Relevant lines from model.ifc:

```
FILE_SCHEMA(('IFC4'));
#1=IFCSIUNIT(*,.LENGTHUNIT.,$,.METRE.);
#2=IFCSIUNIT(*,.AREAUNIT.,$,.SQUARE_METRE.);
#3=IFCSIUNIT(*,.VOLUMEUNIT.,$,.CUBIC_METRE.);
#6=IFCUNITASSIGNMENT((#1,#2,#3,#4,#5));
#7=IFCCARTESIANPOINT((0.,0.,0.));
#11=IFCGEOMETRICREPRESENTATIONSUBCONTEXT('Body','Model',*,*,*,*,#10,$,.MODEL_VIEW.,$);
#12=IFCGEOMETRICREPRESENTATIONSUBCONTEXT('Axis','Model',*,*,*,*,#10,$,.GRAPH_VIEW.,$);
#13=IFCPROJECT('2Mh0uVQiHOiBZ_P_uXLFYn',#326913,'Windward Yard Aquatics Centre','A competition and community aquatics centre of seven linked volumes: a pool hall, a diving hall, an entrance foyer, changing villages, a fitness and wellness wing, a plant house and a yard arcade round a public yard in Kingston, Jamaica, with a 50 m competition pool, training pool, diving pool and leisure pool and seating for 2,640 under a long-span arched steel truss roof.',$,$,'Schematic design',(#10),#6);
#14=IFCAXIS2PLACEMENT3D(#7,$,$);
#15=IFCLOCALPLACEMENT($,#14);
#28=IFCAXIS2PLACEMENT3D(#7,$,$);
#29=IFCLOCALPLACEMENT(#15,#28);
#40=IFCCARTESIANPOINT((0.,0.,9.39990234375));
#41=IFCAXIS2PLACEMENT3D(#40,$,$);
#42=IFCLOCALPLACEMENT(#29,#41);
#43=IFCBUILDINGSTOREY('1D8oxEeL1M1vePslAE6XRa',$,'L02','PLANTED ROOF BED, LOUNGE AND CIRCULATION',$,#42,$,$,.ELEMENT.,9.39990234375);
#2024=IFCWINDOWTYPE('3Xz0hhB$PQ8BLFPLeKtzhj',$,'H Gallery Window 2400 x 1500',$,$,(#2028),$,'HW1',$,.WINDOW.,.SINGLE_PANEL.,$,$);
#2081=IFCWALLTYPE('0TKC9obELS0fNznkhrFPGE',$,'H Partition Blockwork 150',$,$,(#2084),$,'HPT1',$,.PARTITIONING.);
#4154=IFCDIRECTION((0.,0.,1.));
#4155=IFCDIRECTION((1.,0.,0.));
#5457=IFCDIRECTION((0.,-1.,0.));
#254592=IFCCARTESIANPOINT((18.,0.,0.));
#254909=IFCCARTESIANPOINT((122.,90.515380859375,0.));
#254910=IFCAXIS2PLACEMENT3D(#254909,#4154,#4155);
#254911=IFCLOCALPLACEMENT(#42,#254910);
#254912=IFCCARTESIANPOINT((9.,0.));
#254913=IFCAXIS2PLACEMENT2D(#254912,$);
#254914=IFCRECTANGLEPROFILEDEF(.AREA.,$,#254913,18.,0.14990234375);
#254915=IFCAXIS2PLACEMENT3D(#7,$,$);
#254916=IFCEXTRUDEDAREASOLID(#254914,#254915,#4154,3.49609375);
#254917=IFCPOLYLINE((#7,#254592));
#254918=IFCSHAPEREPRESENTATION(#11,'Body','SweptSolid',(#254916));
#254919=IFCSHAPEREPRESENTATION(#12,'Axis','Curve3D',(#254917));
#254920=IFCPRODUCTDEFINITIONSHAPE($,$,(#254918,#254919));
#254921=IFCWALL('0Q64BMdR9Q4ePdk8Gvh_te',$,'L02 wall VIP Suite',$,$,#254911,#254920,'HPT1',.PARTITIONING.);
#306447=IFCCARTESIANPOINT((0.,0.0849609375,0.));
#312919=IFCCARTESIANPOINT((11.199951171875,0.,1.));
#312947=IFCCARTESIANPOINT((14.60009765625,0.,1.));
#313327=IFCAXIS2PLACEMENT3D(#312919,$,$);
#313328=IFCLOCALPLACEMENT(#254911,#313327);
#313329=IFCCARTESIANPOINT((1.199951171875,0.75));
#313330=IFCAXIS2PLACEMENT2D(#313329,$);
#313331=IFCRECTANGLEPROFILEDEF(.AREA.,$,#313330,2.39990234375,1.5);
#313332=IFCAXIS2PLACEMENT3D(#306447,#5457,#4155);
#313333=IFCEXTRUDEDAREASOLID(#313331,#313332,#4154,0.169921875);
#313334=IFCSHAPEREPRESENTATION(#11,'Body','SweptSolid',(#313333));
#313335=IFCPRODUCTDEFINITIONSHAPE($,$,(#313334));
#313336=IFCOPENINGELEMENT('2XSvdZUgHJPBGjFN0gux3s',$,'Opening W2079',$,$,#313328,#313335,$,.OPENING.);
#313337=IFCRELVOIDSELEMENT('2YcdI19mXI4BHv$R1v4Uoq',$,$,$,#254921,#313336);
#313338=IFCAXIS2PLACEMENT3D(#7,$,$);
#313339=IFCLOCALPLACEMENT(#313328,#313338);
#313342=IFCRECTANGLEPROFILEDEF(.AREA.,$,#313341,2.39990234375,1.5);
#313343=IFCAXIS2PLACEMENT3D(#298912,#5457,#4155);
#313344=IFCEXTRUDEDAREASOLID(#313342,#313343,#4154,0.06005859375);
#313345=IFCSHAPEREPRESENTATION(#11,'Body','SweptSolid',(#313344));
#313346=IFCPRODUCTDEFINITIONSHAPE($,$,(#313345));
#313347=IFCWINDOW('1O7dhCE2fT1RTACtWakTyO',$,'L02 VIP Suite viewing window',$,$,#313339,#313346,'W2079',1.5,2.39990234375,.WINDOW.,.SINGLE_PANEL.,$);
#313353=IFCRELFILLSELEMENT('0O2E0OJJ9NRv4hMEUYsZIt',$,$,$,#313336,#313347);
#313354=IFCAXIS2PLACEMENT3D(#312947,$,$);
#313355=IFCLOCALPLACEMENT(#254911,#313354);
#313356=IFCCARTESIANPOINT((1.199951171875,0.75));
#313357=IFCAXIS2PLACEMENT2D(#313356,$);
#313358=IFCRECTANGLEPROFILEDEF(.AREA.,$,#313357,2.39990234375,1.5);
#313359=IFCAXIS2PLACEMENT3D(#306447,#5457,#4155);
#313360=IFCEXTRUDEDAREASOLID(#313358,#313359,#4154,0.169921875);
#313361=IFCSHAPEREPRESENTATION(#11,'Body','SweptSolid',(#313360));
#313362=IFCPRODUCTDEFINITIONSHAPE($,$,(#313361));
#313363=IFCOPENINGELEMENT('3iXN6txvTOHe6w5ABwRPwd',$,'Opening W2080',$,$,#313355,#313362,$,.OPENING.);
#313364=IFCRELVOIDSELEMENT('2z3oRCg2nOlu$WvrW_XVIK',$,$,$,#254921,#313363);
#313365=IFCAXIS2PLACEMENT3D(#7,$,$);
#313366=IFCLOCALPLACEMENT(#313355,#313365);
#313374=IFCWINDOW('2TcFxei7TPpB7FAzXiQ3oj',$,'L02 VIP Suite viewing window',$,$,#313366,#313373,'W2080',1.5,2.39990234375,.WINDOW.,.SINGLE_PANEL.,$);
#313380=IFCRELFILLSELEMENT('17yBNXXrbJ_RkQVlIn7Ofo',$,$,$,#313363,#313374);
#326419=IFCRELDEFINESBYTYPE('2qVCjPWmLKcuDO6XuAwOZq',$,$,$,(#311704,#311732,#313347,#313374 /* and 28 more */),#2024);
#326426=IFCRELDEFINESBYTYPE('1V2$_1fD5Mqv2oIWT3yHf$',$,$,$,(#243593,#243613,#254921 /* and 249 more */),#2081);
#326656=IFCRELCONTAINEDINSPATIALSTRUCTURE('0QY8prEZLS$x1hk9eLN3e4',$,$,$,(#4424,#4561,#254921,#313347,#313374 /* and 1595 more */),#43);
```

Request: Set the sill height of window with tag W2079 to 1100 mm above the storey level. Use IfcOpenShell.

```python
import numpy as np
import ifcopenshell
import ifcopenshell.api.geometry
import ifcopenshell.geom
import ifcopenshell.util.element
import ifcopenshell.util.placement
import ifcopenshell.util.shape
import ifcopenshell.util.unit

model = ifcopenshell.open("model.ifc")
unit_scale = ifcopenshell.util.unit.calculate_unit_scale(model)

window = model.by_guid("1O7dhCE2fT1RTACtWakTyO")
opening = window.FillsVoids[0].RelatingOpeningElement
storey = ifcopenshell.util.element.get_container(window, ifc_class="IfcBuildingStorey")
level = ifcopenshell.util.placement.get_local_placement(storey.ObjectPlacement)[2, 3]

# The opening's origin need not be at the sill, so measure its lowest point.
shape = ifcopenshell.geom.create_shape(ifcopenshell.geom.settings(), opening)
bottom = ifcopenshell.util.shape.get_shape_bottom_elevation(shape, shape.geometry) / unit_scale
dz = level + 1.1 - bottom

shift = np.array([0.0, 0.0, dz])
# The window is placed relative to its opening, so it follows when the opening moves.
matrix = ifcopenshell.util.placement.get_local_placement(opening.ObjectPlacement)
matrix[:3, 3] += shift
ifcopenshell.api.geometry.edit_object_placement(
    model, product=opening, matrix=matrix, is_si=False, should_transform_children=True
)

print(f"moved by {dz * unit_scale:+.3f} m")

model.write("model_edited.ifc")
```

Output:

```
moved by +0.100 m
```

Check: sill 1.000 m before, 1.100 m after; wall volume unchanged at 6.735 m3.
